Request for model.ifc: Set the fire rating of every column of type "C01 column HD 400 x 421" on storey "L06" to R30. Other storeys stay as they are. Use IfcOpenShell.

First a look at what the model holds.

```python
import ifcopenshell
import ifcopenshell.util.element

model = ifcopenshell.open("model.ifc")
print(model.schema)
storey = next(s for s in model.by_type("IfcBuildingStorey") if s.Name == "L06")
columns = [e for e in ifcopenshell.util.element.get_decomposition(storey) if e.is_a("IfcColumn")]
seen = {}
for e in columns:
    element_type = ifcopenshell.util.element.get_type(e)
    key = (element_type.Name if element_type != e and element_type else None, ifcopenshell.util.element.get_pset(e, "Pset_ColumnCommon", "FireRating"))
    seen[key] = seen.get(key, 0) + 1
for (name, value), count in sorted(seen.items(), key=str):
    print(count, "x", name, "|", value)
```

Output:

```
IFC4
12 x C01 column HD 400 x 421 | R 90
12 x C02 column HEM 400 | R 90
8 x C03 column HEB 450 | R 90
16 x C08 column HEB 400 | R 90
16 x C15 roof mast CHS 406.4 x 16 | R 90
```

```python
import ifcopenshell
import ifcopenshell.api.pset
import ifcopenshell.util.element

model = ifcopenshell.open("model.ifc")

storey = next(s for s in model.by_type("IfcBuildingStorey") if s.Name == "L06")
columns = [e for e in ifcopenshell.util.element.get_decomposition(storey) if e.is_a("IfcColumn")]

count = 0
for e in columns:
    element_type = ifcopenshell.util.element.get_type(e)
    if element_type in (None, e) or element_type.Name != "C01 column HD 400 x 421":
        continue
    # add_pset returns the element's existing set when there is one.
    pset = ifcopenshell.api.pset.add_pset(model, product=e, name="Pset_ColumnCommon")
    ifcopenshell.api.pset.edit_pset(model, pset=pset, properties={"FireRating": "R30"})
    count += 1

print(count, "columns updated")

model.write("model_rev.ifc")
```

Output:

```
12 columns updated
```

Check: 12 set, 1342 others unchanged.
